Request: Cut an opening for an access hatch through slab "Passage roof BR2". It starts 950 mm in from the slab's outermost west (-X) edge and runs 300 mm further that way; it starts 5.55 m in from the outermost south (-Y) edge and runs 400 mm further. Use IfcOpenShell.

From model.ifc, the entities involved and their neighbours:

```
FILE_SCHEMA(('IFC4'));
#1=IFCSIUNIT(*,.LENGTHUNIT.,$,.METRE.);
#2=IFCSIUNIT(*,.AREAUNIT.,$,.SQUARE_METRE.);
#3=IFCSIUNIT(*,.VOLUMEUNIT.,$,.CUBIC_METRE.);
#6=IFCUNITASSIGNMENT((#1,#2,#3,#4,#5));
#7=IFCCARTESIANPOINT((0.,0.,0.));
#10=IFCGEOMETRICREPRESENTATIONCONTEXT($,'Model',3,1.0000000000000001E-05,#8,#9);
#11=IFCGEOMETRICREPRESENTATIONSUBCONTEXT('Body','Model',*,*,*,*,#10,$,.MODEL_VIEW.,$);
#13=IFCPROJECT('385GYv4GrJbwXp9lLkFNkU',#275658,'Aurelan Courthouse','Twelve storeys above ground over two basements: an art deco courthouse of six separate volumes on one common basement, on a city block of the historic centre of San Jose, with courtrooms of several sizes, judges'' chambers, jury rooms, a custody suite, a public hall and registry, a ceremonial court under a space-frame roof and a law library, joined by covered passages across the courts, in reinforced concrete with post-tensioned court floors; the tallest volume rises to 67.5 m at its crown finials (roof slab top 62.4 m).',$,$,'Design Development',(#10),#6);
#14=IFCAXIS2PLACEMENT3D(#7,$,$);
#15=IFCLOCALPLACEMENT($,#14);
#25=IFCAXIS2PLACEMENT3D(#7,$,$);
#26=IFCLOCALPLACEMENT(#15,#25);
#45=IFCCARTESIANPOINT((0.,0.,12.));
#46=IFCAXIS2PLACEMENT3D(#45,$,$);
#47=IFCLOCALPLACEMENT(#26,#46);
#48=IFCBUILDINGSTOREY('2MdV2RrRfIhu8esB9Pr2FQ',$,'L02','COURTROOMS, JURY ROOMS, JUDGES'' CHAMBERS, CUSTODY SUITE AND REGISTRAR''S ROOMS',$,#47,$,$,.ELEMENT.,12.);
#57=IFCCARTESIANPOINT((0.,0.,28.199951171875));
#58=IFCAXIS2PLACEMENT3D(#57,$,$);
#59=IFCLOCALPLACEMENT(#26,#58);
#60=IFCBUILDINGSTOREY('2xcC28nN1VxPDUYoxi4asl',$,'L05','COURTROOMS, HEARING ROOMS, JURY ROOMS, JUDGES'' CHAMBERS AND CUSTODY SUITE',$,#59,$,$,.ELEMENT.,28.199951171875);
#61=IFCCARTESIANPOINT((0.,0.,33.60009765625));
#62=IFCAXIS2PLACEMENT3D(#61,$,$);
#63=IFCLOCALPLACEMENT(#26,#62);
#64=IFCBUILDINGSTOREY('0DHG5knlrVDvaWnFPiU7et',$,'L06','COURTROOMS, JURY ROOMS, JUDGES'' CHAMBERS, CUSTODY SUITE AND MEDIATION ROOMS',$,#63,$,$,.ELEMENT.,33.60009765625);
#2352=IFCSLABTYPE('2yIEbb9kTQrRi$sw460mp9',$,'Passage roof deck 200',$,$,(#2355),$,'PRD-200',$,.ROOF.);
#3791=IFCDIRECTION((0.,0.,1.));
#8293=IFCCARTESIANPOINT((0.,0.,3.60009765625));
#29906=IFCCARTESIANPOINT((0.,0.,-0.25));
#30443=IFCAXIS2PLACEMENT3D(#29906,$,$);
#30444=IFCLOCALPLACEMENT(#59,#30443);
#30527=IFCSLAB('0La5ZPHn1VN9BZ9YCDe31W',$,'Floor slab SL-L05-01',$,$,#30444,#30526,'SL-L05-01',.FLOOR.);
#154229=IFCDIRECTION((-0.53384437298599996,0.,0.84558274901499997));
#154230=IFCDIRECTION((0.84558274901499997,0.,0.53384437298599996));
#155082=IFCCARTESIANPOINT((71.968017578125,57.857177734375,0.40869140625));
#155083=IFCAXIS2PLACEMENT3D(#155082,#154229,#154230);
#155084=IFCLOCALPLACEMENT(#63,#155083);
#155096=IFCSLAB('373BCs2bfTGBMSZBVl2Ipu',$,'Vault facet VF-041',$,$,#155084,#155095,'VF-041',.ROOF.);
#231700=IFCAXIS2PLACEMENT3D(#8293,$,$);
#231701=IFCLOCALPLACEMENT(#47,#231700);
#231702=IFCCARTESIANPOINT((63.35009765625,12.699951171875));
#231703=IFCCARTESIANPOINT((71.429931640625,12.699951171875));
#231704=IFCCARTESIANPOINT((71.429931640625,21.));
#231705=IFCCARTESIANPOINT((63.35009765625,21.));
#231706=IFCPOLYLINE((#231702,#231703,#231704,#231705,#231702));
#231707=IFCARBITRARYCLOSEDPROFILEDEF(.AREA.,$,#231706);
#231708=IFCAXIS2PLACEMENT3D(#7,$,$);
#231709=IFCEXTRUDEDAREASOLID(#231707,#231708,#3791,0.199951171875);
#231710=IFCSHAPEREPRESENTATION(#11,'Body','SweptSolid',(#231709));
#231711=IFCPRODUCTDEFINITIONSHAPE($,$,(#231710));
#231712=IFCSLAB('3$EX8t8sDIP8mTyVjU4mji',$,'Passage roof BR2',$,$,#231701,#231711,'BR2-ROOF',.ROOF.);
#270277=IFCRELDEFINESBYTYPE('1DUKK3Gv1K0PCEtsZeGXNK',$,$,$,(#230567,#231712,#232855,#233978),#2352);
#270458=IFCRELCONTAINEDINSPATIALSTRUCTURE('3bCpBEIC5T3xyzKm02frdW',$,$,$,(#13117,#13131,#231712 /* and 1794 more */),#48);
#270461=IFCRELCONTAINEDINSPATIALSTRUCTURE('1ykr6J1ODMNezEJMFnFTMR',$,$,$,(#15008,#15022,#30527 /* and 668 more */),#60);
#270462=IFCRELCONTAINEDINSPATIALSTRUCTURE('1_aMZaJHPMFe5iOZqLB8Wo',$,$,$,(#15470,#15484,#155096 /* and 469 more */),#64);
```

```python
import numpy as np
import ifcopenshell
import ifcopenshell.api.feature
import ifcopenshell.api.geometry
import ifcopenshell.api.root
import ifcopenshell.geom
import ifcopenshell.util.placement
import ifcopenshell.util.representation
import ifcopenshell.util.shape
import ifcopenshell.util.unit

model = ifcopenshell.open("model.ifc")
unit_scale = ifcopenshell.util.unit.calculate_unit_scale(model)
settings = ifcopenshell.geom.settings()


def volume(element):
    """Net volume in cubic metres, openings subtracted."""
    shape = ifcopenshell.geom.create_shape(settings, element)
    return ifcopenshell.util.shape.get_volume(shape.geometry)


slab = model.by_guid("3$EX8t8sDIP8mTyVjU4mji")
before = volume(slab)

# Extent in the slab's own axes, in metres. The edges named are its -X and -Y sides.
slab_shape = ifcopenshell.geom.create_shape(settings, slab)
vertices = ifcopenshell.util.shape.get_vertices(slab_shape.geometry)
x_min, y_min, bottom = vertices.min(axis=0)
top = vertices[:, 2].max()

opening = ifcopenshell.api.root.create_entity(model, ifc_class="IfcOpeningElement", name="Access hatch opening", predefined_type="OPENING")
context = ifcopenshell.util.representation.get_context(model, "Model", "Body", "MODEL_VIEW")
width, depth = 0.3, 0.4
outline = [(0.0, 0.0), (width, 0.0), (width, depth), (0.0, depth), (0.0, 0.0)]
# Overshoot both faces by 50 mm so the cut is clean.
shape = ifcopenshell.api.geometry.add_slab_representation(
    model, context=context, depth=top - bottom + 0.1, polyline=outline
)
ifcopenshell.api.geometry.assign_representation(model, product=opening, representation=shape)

matrix = ifcopenshell.util.placement.get_local_placement(slab.ObjectPlacement)
matrix[:, 3] = matrix @ np.append(np.array([x_min + 0.95, y_min + 5.55, bottom - 0.05]) / unit_scale, 1.0)
ifcopenshell.api.geometry.edit_object_placement(model, product=opening, matrix=matrix, is_si=False)
ifcopenshell.api.feature.add_feature(model, feature=opening, element=slab)

after = volume(slab)

print(f"slab volume {before:.3f} -> {after:.3f} m3")

model.write("model-out.ifc")
```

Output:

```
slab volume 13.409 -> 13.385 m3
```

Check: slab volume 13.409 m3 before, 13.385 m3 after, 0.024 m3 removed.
